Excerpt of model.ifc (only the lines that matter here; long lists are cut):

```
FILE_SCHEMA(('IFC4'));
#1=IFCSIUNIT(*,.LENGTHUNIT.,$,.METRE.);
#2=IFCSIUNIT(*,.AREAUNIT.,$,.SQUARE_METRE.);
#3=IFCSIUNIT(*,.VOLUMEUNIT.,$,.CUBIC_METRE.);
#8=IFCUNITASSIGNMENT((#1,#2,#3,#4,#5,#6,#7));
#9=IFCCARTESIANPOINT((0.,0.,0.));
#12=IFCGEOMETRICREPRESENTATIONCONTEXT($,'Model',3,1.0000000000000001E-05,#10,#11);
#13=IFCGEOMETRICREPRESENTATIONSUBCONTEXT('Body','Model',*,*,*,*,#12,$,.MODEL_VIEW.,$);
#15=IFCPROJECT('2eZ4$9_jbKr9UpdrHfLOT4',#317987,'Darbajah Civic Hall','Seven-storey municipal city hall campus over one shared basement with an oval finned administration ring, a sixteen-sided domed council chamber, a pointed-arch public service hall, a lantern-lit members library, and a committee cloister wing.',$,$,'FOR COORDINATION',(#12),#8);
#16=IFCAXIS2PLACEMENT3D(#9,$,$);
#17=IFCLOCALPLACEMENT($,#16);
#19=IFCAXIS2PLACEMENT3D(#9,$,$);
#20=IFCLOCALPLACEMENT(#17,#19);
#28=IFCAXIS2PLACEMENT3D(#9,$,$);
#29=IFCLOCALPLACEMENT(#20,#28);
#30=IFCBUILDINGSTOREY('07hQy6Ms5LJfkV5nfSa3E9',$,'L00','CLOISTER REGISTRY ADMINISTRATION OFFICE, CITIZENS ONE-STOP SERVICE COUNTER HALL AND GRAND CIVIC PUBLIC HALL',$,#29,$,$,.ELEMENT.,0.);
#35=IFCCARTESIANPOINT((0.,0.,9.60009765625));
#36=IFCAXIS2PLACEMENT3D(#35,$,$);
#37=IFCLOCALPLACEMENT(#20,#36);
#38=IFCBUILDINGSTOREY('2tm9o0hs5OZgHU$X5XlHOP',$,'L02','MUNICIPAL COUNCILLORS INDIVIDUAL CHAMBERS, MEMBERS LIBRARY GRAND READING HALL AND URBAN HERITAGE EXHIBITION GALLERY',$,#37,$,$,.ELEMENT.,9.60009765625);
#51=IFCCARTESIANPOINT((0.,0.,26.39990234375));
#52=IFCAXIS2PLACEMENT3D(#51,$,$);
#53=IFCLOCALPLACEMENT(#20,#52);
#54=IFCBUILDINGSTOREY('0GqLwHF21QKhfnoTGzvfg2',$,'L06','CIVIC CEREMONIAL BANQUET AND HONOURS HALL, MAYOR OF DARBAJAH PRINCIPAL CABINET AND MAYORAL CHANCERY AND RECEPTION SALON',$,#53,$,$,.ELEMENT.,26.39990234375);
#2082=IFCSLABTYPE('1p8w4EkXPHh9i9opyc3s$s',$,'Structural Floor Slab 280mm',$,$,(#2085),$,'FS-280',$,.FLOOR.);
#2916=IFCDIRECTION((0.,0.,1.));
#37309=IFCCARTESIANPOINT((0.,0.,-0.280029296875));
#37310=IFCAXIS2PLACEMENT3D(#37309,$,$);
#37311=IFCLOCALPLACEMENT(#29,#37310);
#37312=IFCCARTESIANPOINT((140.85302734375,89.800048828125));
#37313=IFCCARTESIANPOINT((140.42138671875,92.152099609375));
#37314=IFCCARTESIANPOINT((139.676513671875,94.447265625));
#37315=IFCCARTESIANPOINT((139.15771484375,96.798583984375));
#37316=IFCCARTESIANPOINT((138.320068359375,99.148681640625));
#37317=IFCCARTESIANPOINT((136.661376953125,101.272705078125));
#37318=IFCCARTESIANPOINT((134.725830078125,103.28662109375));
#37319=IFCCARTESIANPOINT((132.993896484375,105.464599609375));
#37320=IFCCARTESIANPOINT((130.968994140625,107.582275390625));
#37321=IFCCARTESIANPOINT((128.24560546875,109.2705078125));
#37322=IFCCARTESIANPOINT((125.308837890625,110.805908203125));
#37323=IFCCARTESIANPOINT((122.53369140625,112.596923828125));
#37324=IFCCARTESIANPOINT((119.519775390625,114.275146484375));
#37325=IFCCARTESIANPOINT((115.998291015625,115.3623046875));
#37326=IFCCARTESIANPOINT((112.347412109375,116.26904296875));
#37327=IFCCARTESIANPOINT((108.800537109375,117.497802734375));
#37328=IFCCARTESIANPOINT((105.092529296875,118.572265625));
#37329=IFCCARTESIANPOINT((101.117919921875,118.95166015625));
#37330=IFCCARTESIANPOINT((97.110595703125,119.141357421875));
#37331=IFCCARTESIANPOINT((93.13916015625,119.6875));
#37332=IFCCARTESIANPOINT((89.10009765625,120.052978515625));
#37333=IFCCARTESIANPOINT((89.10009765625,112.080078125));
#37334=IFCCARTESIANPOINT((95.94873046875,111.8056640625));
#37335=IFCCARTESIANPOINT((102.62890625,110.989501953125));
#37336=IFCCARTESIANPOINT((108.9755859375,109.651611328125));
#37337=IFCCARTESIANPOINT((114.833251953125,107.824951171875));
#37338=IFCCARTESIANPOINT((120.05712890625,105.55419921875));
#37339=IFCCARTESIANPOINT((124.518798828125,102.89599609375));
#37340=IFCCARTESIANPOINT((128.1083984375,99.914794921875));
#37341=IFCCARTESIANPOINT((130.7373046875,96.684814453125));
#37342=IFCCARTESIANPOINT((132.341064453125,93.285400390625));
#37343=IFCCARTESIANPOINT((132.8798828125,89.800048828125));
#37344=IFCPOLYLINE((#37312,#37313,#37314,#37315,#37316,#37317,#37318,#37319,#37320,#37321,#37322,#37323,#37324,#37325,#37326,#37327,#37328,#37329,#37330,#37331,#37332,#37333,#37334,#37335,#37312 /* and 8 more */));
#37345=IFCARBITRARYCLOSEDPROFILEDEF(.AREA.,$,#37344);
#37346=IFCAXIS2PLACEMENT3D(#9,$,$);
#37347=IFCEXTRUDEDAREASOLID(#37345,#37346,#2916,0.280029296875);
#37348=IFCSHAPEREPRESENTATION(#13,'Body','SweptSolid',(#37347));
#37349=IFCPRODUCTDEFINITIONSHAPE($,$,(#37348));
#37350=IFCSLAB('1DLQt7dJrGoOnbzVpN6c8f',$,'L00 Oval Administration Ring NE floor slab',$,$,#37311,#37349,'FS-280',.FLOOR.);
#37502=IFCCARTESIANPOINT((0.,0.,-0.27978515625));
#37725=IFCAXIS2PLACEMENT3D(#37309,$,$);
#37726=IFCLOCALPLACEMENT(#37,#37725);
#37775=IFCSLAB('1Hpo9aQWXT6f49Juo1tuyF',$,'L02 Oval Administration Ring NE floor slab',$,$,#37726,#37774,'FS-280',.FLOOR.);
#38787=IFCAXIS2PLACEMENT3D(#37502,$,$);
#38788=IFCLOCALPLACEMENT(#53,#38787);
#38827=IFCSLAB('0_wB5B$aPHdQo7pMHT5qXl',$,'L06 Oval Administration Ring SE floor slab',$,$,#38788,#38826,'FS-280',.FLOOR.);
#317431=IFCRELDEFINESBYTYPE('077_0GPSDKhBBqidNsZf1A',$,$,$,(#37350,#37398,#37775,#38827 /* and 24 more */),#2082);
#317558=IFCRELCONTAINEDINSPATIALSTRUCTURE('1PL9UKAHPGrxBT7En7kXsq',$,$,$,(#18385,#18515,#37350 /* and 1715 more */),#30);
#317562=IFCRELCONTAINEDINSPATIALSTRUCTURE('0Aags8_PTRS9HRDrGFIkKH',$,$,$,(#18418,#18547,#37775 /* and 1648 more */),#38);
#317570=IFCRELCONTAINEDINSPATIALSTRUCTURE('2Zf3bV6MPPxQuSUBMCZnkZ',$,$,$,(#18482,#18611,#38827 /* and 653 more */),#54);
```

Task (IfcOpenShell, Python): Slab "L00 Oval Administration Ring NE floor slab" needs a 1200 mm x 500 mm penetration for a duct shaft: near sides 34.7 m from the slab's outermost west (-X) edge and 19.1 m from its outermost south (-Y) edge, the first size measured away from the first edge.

```python
import numpy as np
import ifcopenshell
import ifcopenshell.api.feature
import ifcopenshell.api.geometry
import ifcopenshell.api.root
import ifcopenshell.geom
import ifcopenshell.util.placement
import ifcopenshell.util.representation
import ifcopenshell.util.shape
import ifcopenshell.util.unit

model = ifcopenshell.open("model.ifc")
unit_scale = ifcopenshell.util.unit.calculate_unit_scale(model)
settings = ifcopenshell.geom.settings()


def volume(element):
    """Net volume in cubic metres, openings subtracted."""
    shape = ifcopenshell.geom.create_shape(settings, element)
    return ifcopenshell.util.shape.get_volume(shape.geometry)


slab = model.by_guid("1DLQt7dJrGoOnbzVpN6c8f")
before = volume(slab)

# Extent in the slab's own axes, in metres. The edges named are its -X and -Y sides.
slab_shape = ifcopenshell.geom.create_shape(settings, slab)
vertices = ifcopenshell.util.shape.get_vertices(slab_shape.geometry)
x_min, y_min, bottom = vertices.min(axis=0)
top = vertices[:, 2].max()

opening = ifcopenshell.api.root.create_entity(model, ifc_class="IfcOpeningElement", name="Duct shaft opening", predefined_type="OPENING")
context = ifcopenshell.util.representation.get_context(model, "Model", "Body", "MODEL_VIEW")
width, depth = 1.2, 0.5
outline = [(0.0, 0.0), (width, 0.0), (width, depth), (0.0, depth), (0.0, 0.0)]
# Overshoot both faces by 50 mm so the cut is clean.
shape = ifcopenshell.api.geometry.add_slab_representation(
    model, context=context, depth=top - bottom + 0.1, polyline=outline
)
ifcopenshell.api.geometry.assign_representation(model, product=opening, representation=shape)

matrix = ifcopenshell.util.placement.get_local_placement(slab.ObjectPlacement)
matrix[:, 3] = matrix @ np.append(np.array([x_min + 34.7, y_min + 19.1, bottom - 0.05]) / unit_scale, 1.0)
ifcopenshell.api.geometry.edit_object_placement(model, product=opening, matrix=matrix, is_si=False)
ifcopenshell.api.feature.add_feature(model, feature=opening, element=slab)

after = volume(slab)

print(f"slab volume {before:.3f} -> {after:.3f} m3")

model.write("model_v2.ifc")
```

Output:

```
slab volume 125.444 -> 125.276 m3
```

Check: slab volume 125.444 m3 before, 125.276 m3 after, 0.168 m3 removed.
